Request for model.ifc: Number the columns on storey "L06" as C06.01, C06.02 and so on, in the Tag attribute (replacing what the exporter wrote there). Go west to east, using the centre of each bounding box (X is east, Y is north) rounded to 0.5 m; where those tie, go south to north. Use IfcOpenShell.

First a look at what the model holds.

```python
import ifcopenshell
import ifcopenshell.util.element
import ifcopenshell.util.placement

model = ifcopenshell.open("model.ifc")
print(model.schema)
storey = next(s for s in model.by_type("IfcBuildingStorey") if s.Name == "L06")
columns = [e for e in ifcopenshell.util.element.get_decomposition(storey) if e.is_a("IfcColumn")]
for e in sorted(columns, key=lambda e: e.id()):
    origin = ifcopenshell.util.placement.get_local_placement(e.ObjectPlacement)[:3, 3]
    print(e.id(), e.Tag, e.Name, origin.round(2) + 0.0, sep=" | ")
```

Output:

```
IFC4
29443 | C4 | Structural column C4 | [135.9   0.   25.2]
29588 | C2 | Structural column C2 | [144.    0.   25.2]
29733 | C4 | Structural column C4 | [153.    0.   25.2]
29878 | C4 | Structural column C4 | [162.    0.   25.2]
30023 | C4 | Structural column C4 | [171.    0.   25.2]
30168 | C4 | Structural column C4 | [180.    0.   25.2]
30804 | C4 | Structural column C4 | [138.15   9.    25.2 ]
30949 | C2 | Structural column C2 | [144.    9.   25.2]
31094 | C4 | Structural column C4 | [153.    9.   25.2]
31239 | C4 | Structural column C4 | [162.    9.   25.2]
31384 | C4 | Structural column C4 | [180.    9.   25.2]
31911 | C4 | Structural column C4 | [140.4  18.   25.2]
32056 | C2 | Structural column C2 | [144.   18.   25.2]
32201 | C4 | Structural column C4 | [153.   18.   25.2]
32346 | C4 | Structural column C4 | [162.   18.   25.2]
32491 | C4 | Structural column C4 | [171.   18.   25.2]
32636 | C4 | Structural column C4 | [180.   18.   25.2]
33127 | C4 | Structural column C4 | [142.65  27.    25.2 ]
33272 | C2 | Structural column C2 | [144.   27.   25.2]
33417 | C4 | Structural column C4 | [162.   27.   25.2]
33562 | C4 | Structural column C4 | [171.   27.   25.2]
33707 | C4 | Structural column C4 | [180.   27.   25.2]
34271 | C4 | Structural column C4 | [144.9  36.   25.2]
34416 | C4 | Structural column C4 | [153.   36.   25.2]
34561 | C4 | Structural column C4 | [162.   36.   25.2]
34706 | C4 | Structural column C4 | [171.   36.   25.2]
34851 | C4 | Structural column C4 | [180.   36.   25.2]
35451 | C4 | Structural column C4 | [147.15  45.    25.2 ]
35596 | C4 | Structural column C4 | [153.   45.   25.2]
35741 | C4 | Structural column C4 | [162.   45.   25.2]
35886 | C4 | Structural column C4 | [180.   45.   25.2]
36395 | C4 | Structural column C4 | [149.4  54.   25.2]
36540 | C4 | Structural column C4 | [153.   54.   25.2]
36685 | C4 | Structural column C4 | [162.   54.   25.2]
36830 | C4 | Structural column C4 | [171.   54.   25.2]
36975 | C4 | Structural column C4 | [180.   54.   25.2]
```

```python
import ifcopenshell
import ifcopenshell.geom
import ifcopenshell.util.element
import ifcopenshell.util.shape

model = ifcopenshell.open("model.ifc")
settings = ifcopenshell.geom.settings()
settings.set("use-world-coords", True)


def centre(element):
    shape = ifcopenshell.geom.create_shape(settings, element)
    return ifcopenshell.util.shape.get_bbox_centroid(shape.geometry)


storey = next(s for s in model.by_type("IfcBuildingStorey") if s.Name == "L06")
columns = [e for e in ifcopenshell.util.element.get_decomposition(storey) if e.is_a("IfcColumn")]

# Insertion points can sit at a corner or the storey origin, so sort by the geometry (in metres).
centres = {e: centre(e) for e in columns}
columns.sort(key=lambda e: (round(centres[e][0] / 0.5), centres[e][1]))

for i, e in enumerate(columns, start=1):
    number = f"C06.{i:02d}"
    e.Tag = number
    print(e.id(), number)

model.write("model-out.ifc")
```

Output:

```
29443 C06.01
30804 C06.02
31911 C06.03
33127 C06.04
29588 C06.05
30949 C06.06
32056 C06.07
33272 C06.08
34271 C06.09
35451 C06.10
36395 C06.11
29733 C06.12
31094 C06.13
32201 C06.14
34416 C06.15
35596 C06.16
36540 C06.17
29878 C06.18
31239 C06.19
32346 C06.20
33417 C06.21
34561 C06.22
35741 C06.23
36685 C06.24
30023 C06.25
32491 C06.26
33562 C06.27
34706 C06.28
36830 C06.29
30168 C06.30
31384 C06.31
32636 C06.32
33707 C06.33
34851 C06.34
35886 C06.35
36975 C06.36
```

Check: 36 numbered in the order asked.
